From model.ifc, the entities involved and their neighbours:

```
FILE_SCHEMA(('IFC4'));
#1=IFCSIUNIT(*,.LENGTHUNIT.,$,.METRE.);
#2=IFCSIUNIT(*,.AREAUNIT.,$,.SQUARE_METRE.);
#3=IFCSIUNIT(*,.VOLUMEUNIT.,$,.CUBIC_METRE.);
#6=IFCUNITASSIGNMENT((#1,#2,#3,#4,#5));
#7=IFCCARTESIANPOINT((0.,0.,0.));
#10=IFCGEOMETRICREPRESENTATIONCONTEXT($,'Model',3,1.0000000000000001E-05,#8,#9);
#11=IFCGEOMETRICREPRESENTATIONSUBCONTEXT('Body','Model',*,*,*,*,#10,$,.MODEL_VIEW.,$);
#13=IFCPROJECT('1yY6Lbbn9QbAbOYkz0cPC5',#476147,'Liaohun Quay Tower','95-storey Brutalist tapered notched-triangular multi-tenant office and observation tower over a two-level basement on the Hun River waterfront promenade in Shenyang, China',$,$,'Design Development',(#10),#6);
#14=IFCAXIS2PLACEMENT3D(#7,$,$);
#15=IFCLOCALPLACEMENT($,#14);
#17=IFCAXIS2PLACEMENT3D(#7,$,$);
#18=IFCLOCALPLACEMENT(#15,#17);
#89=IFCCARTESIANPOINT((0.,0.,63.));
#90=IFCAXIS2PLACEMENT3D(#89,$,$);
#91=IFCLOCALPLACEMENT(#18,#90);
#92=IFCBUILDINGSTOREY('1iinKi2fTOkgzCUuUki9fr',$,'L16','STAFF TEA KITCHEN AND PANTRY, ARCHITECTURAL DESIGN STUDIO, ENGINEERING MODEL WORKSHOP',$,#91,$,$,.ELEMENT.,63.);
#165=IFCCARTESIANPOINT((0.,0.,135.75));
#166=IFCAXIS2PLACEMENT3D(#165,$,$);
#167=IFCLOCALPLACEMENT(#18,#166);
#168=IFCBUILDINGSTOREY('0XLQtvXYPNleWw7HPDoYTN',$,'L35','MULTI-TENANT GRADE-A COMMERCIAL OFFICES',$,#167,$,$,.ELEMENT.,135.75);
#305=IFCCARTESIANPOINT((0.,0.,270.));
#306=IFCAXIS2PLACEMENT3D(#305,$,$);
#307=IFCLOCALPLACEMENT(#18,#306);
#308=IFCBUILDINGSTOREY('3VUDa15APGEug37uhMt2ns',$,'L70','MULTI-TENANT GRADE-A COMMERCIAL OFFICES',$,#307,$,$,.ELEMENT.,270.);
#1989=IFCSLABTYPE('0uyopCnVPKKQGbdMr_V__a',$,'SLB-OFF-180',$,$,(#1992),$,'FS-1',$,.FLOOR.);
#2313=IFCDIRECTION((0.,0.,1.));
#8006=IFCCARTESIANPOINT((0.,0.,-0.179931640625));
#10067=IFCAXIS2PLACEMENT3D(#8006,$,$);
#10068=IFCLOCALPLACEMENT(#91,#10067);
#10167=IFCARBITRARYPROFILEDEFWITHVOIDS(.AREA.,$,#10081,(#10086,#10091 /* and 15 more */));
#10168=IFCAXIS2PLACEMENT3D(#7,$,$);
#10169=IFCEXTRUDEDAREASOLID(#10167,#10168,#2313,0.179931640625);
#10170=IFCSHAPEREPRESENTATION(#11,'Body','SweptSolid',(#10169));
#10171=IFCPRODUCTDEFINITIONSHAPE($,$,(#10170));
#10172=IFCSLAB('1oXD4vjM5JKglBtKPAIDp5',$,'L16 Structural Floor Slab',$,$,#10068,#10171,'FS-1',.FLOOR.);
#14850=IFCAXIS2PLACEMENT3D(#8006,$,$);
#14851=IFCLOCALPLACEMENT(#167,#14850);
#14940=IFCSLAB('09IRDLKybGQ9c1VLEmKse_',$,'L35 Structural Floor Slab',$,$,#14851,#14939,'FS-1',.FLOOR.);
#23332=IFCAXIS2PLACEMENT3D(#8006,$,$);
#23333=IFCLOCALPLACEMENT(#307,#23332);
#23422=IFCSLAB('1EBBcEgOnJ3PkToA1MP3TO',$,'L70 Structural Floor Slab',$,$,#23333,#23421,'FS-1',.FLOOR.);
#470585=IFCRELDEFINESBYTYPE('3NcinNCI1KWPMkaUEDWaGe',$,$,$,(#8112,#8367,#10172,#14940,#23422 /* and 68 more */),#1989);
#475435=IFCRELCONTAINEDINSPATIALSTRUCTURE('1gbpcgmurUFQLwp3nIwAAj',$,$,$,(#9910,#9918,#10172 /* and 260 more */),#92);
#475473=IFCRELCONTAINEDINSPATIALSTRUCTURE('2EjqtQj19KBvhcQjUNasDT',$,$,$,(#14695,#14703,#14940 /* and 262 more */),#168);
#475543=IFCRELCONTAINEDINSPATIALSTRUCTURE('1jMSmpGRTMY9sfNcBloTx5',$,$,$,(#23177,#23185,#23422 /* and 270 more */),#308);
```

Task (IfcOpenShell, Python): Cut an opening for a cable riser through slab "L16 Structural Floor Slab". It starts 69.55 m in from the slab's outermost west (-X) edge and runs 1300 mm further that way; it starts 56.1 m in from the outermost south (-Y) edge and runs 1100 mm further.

```python
import numpy as np
import ifcopenshell
import ifcopenshell.api.feature
import ifcopenshell.api.geometry
import ifcopenshell.api.root
import ifcopenshell.geom
import ifcopenshell.util.placement
import ifcopenshell.util.representation
import ifcopenshell.util.shape
import ifcopenshell.util.unit

model = ifcopenshell.open("model.ifc")
unit_scale = ifcopenshell.util.unit.calculate_unit_scale(model)
settings = ifcopenshell.geom.settings()


def volume(element):
    """Net volume in cubic metres, openings subtracted."""
    shape = ifcopenshell.geom.create_shape(settings, element)
    return ifcopenshell.util.shape.get_volume(shape.geometry)


slab = model.by_guid("1oXD4vjM5JKglBtKPAIDp5")
before = volume(slab)

# Extent in the slab's own axes, in metres. The edges named are its -X and -Y sides.
slab_shape = ifcopenshell.geom.create_shape(settings, slab)
vertices = ifcopenshell.util.shape.get_vertices(slab_shape.geometry)
x_min, y_min, bottom = vertices.min(axis=0)
top = vertices[:, 2].max()

opening = ifcopenshell.api.root.create_entity(model, ifc_class="IfcOpeningElement", name="Cable riser opening", predefined_type="OPENING")
context = ifcopenshell.util.representation.get_context(model, "Model", "Body", "MODEL_VIEW")
width, depth = 1.3, 1.1
outline = [(0.0, 0.0), (width, 0.0), (width, depth), (0.0, depth), (0.0, 0.0)]
# Overshoot both faces by 50 mm so the cut is clean.
shape = ifcopenshell.api.geometry.add_slab_representation(
    model, context=context, depth=top - bottom + 0.1, polyline=outline
)
ifcopenshell.api.geometry.assign_representation(model, product=opening, representation=shape)

matrix = ifcopenshell.util.placement.get_local_placement(slab.ObjectPlacement)
matrix[:, 3] = matrix @ np.append(np.array([x_min + 69.55, y_min + 56.1, bottom - 0.05]) / unit_scale, 1.0)
ifcopenshell.api.geometry.edit_object_placement(model, product=opening, matrix=matrix, is_si=False)
ifcopenshell.api.feature.add_feature(model, feature=opening, element=slab)

after = volume(slab)

print(f"slab volume {before:.3f} -> {after:.3f} m3")

model.write("model_edited.ifc")
```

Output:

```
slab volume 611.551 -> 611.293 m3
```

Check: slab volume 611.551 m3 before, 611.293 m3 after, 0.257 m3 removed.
